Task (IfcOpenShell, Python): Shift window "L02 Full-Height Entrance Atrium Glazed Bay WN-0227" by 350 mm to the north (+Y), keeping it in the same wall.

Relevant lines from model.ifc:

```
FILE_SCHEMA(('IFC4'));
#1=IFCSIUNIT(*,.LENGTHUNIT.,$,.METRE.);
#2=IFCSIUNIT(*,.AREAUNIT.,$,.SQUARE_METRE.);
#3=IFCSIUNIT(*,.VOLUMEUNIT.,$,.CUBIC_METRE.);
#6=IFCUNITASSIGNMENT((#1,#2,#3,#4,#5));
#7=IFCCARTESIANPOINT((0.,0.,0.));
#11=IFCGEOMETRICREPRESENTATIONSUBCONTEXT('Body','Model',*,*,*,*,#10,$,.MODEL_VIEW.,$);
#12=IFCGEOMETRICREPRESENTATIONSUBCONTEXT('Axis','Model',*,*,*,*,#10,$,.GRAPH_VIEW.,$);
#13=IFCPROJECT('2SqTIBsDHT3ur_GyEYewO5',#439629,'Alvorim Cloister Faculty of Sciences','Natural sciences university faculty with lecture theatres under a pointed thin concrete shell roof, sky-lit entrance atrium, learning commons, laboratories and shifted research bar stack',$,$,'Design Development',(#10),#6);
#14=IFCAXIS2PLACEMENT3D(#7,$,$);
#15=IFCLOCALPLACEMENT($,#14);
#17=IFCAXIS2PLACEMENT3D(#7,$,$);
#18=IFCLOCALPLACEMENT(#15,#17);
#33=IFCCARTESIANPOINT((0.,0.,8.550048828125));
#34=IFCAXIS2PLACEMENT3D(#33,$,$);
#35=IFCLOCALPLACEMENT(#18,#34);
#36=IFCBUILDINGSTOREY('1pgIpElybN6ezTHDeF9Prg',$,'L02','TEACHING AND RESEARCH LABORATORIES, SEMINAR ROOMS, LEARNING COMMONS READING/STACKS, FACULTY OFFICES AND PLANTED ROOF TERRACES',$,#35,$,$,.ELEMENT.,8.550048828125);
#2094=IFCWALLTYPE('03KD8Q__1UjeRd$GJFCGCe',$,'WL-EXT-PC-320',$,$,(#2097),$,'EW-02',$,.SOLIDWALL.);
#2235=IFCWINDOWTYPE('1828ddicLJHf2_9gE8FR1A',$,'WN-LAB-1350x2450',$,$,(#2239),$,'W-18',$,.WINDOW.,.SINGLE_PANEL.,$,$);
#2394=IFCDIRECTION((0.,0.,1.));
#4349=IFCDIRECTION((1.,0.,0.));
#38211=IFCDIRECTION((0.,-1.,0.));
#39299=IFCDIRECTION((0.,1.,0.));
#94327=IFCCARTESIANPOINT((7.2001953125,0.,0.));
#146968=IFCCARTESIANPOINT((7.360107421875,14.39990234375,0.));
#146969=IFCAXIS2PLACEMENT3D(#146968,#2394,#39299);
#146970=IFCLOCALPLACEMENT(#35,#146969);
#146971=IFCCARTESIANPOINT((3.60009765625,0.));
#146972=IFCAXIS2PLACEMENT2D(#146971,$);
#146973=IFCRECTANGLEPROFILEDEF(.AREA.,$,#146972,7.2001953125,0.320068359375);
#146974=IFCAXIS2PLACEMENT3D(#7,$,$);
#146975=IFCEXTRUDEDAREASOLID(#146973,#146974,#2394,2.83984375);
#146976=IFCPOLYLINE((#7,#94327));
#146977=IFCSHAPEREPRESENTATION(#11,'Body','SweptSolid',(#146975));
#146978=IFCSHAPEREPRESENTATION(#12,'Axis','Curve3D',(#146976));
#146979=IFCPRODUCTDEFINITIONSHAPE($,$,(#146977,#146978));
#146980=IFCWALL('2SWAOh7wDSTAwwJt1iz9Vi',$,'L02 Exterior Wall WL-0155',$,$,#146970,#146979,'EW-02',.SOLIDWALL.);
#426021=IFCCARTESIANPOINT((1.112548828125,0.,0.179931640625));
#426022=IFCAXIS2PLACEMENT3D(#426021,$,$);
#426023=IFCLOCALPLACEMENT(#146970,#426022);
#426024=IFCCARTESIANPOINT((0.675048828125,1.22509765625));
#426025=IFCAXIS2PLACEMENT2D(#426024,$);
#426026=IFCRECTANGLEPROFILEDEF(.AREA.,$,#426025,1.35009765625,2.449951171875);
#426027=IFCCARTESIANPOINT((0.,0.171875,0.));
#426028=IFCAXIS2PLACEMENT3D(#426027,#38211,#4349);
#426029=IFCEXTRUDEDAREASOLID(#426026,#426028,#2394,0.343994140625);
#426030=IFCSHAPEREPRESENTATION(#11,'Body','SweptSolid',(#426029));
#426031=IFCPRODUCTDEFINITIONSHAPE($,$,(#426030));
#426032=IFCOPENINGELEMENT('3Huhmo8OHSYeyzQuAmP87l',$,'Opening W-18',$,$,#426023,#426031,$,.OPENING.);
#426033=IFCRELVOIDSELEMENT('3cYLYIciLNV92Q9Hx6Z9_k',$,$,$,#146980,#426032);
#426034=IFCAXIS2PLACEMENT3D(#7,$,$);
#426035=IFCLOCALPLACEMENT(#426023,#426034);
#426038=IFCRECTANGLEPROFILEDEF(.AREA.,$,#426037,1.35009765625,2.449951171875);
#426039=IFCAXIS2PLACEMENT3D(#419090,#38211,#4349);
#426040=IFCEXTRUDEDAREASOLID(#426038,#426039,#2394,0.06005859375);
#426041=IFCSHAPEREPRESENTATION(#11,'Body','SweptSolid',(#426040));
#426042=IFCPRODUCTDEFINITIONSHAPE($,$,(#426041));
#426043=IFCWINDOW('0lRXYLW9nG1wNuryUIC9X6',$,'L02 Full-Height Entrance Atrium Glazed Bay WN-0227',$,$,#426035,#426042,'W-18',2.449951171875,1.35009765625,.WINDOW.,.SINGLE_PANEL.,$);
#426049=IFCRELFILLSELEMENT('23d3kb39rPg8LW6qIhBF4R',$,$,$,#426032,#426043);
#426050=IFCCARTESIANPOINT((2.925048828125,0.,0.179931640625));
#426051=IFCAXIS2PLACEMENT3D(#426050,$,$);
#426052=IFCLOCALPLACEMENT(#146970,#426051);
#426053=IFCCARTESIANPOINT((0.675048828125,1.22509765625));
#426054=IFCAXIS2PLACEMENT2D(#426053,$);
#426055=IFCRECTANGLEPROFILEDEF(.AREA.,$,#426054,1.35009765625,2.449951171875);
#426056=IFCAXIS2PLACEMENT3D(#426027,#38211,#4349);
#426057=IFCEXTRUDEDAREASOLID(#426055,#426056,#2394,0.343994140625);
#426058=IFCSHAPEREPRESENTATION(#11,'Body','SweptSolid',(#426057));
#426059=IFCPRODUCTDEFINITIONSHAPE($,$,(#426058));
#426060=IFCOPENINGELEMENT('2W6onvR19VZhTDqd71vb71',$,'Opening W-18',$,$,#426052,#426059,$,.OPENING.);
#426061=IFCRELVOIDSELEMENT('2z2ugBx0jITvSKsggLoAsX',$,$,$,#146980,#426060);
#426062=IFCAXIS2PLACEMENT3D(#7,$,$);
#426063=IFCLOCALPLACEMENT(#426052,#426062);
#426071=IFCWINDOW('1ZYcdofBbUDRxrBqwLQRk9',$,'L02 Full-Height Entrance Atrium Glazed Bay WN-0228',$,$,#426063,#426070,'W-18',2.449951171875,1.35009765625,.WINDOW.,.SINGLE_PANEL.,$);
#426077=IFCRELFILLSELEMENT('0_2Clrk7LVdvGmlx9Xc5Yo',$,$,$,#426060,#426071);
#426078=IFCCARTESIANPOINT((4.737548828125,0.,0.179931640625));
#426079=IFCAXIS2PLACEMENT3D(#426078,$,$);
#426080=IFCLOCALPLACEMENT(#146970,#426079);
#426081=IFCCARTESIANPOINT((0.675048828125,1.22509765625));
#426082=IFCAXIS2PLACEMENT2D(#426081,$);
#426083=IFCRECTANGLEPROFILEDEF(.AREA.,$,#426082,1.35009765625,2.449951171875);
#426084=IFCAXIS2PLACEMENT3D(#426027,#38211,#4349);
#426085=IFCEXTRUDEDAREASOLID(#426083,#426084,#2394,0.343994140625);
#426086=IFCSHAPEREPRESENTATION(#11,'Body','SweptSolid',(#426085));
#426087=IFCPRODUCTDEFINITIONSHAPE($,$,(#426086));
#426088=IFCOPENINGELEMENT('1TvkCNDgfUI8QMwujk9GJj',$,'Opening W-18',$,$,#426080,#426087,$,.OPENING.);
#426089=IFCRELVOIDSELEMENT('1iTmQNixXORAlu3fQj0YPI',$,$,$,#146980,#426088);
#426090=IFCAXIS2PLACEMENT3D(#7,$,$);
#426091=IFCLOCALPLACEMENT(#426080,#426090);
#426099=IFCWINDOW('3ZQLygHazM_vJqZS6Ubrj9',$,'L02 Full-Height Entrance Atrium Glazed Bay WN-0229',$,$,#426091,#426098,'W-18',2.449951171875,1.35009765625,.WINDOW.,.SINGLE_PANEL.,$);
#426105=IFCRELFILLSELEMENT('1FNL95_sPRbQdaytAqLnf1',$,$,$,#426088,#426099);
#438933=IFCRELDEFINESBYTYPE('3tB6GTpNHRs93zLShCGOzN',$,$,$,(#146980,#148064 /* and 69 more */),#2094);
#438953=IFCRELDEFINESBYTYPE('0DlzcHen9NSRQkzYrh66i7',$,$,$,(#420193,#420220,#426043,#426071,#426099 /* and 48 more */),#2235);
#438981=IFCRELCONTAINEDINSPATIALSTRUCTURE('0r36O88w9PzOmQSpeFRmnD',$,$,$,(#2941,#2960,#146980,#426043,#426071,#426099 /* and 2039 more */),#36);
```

```python
import ifcopenshell
import ifcopenshell.api.geometry
import ifcopenshell.util.placement
import ifcopenshell.util.unit

model = ifcopenshell.open("model.ifc")
unit_scale = ifcopenshell.util.unit.calculate_unit_scale(model)

window = model.by_guid("0lRXYLW9nG1wNuryUIC9X6")
opening = window.FillsVoids[0].RelatingOpeningElement
wall = opening.VoidsElements[0].RelatingBuildingElement

wall_matrix = ifcopenshell.util.placement.get_local_placement(wall.ObjectPlacement)
shift = wall_matrix[:3, 0] * 0.35 / unit_scale
before = ifcopenshell.util.placement.get_local_placement(window.ObjectPlacement)[:3, 3].copy()

# The window is placed relative to its opening, so it follows when the opening moves.
matrix = ifcopenshell.util.placement.get_local_placement(opening.ObjectPlacement)
matrix[:3, 3] += shift
ifcopenshell.api.geometry.edit_object_placement(
    model, product=opening, matrix=matrix, is_si=False, should_transform_children=True
)

after = ifcopenshell.util.placement.get_local_placement(window.ObjectPlacement)[:3, 3]
print("window moved by", (after - before).round(3) + 0.0)

model.write("model-out.ifc")
```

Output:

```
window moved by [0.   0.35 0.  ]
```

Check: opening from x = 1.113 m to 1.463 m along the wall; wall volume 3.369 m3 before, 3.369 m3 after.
